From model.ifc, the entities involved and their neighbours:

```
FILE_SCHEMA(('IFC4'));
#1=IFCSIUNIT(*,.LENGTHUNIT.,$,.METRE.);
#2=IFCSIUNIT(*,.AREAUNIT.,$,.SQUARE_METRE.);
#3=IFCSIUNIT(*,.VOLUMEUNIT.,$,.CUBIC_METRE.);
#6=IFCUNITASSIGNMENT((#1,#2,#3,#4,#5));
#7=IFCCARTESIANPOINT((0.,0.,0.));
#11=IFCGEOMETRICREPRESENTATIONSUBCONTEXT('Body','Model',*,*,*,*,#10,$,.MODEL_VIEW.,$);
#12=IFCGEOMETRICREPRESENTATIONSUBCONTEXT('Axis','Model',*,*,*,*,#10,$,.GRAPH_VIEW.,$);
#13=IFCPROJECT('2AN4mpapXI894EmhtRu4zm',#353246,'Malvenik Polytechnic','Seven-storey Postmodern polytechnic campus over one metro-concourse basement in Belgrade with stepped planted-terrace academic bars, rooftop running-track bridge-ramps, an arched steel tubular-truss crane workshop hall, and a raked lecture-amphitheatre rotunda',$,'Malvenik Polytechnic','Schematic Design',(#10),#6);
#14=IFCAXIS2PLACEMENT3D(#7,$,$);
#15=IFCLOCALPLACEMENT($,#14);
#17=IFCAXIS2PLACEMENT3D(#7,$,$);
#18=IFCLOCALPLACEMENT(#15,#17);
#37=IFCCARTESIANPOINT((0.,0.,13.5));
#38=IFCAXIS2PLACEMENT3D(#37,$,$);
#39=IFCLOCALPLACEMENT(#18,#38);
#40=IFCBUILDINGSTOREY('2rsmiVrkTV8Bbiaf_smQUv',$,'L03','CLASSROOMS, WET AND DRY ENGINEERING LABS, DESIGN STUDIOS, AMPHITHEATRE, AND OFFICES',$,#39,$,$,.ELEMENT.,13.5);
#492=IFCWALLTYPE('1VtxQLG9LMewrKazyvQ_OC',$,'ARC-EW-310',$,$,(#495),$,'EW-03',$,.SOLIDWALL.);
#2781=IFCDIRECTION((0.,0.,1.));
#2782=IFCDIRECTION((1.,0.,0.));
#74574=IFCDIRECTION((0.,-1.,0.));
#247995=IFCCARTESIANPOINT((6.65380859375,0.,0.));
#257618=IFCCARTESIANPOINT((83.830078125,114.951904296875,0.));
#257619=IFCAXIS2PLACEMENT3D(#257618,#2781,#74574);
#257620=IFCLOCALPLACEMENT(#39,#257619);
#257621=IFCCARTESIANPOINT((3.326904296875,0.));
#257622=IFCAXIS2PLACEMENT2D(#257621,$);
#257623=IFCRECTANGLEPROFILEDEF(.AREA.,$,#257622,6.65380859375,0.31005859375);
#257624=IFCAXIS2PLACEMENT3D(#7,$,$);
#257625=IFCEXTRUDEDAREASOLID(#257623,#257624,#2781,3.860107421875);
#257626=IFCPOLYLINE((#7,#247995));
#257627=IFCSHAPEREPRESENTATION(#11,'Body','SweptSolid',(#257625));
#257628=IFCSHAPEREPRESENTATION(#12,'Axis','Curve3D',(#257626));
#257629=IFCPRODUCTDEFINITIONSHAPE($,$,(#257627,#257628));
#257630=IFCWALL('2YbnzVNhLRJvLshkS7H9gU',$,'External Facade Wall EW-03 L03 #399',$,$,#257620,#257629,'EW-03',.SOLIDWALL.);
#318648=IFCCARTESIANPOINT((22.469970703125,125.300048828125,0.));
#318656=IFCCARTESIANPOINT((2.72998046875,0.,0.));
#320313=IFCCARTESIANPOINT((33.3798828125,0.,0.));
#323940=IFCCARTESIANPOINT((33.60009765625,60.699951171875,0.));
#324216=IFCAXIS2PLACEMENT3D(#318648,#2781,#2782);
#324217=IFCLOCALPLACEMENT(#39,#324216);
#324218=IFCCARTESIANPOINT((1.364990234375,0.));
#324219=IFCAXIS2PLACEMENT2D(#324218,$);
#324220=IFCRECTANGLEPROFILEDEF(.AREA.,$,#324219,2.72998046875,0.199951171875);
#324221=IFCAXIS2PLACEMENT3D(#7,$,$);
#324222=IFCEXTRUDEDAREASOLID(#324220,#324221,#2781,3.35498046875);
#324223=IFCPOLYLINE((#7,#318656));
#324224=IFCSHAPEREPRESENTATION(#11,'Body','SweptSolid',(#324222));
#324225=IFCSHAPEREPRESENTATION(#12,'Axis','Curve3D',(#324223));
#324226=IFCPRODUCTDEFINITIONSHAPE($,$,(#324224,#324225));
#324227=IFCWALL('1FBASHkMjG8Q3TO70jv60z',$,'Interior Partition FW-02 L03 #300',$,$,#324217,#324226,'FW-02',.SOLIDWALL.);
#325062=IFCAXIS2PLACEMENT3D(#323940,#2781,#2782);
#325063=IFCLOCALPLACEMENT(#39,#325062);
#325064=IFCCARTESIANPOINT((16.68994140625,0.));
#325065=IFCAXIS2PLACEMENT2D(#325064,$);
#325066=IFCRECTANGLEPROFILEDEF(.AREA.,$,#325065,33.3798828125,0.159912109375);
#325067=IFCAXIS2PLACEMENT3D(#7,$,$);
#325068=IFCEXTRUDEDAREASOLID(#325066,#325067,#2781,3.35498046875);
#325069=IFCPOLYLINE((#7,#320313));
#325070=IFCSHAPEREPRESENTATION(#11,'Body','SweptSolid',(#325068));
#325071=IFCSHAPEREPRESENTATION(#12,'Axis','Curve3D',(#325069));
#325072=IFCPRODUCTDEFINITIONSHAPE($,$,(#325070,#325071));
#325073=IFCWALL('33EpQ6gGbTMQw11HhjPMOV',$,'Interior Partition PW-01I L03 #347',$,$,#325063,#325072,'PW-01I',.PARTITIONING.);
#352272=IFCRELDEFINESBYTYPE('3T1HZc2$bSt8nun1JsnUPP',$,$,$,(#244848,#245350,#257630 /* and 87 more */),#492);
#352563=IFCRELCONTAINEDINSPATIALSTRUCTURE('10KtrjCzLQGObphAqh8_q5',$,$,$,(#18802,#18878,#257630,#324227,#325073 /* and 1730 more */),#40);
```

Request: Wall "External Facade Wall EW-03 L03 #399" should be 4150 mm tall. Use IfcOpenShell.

```python
import ifcopenshell
import ifcopenshell.geom
import ifcopenshell.util.representation
import ifcopenshell.util.shape

model = ifcopenshell.open("model.ifc")
settings = ifcopenshell.geom.settings()


def volume(element):
    """Net volume in cubic metres, openings subtracted."""
    shape = ifcopenshell.geom.create_shape(settings, element)
    return ifcopenshell.util.shape.get_volume(shape.geometry)


wall = model.by_guid("2YbnzVNhLRJvLshkS7H9gU")
before = volume(wall)

body = ifcopenshell.util.representation.get_representation(wall, "Model", "Body")
solid = body.Items[0]
old_height = solid.Depth
solid.Depth = 4.15
after = volume(wall)

print(f"height {old_height:g} -> {solid.Depth:g}, volume {before:.3f} -> {after:.3f} m3")

model.write("model_edited.ifc")
```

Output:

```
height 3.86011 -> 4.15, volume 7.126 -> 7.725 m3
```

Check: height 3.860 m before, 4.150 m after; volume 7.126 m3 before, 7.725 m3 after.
